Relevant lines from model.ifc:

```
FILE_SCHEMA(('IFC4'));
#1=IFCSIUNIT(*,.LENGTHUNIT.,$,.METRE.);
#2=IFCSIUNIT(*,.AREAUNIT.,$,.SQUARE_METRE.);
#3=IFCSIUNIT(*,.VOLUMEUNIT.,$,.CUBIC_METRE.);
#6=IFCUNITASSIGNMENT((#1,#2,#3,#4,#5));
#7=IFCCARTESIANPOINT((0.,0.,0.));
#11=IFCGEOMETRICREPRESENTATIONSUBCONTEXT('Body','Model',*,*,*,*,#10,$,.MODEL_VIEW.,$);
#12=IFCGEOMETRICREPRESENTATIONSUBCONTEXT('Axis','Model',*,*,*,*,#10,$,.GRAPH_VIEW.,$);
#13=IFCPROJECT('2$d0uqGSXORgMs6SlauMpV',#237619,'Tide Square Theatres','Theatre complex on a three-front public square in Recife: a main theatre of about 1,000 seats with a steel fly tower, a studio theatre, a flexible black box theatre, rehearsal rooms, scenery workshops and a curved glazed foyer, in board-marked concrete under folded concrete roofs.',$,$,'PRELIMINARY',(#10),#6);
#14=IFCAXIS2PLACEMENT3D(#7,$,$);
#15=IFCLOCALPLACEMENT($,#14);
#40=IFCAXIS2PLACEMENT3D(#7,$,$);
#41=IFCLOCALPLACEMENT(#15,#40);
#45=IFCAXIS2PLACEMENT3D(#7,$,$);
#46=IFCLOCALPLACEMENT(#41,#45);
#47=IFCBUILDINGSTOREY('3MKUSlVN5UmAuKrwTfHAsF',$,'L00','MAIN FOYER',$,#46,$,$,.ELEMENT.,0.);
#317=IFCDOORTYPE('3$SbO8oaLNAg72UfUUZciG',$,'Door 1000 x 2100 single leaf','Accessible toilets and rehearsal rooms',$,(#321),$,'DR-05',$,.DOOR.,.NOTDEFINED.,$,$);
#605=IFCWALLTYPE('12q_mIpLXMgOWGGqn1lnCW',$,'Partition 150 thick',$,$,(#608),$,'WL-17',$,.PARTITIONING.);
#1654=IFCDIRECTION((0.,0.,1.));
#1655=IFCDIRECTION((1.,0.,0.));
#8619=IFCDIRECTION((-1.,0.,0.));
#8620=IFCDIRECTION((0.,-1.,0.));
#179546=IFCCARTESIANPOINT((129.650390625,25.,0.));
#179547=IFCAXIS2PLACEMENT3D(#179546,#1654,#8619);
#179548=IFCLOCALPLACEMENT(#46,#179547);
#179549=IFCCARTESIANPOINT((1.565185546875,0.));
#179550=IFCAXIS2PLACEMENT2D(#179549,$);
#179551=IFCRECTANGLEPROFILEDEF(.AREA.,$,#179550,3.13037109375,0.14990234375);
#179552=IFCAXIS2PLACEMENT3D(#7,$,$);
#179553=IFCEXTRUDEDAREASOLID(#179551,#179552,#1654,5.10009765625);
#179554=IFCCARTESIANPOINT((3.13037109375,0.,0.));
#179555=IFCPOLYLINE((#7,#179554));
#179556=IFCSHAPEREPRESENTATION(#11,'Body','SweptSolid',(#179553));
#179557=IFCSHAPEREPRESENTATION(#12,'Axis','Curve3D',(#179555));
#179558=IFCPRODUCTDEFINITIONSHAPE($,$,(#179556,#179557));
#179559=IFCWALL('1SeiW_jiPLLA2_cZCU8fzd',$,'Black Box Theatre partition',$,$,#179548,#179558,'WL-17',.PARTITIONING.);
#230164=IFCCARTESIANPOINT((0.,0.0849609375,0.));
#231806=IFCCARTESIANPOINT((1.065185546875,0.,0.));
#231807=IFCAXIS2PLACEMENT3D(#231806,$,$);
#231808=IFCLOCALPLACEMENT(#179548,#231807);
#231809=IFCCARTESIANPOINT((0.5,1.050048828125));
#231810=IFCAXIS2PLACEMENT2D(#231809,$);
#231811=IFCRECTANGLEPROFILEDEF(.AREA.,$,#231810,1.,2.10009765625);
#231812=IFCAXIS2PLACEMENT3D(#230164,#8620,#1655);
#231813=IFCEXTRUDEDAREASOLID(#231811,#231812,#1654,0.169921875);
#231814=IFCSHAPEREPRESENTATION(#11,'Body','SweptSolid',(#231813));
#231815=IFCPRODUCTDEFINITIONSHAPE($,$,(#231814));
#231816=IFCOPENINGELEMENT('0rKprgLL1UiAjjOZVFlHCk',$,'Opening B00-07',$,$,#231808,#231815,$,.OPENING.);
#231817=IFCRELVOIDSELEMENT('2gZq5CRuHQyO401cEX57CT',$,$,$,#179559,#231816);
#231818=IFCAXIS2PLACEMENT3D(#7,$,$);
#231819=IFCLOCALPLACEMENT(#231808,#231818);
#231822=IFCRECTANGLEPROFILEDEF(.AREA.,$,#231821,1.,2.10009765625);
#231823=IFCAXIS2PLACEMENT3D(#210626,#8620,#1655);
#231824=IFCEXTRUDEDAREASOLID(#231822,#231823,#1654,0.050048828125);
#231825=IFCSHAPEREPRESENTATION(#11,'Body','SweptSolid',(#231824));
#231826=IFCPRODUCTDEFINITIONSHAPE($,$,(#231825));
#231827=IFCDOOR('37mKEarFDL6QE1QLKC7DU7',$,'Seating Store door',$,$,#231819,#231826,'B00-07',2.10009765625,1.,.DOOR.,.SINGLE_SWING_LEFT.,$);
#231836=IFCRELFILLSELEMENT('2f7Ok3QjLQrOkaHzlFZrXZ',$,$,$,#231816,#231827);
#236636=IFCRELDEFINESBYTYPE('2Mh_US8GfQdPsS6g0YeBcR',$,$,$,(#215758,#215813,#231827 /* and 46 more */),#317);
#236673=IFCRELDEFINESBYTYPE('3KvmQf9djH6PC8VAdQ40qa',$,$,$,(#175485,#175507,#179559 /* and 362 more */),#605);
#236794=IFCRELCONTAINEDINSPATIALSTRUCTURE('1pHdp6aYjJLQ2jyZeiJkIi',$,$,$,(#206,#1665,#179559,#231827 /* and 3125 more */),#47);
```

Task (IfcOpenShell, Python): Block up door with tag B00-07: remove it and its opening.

```python
import ifcopenshell
import ifcopenshell.api.feature
import ifcopenshell.api.root
import ifcopenshell.geom
import ifcopenshell.util.shape

model = ifcopenshell.open("model.ifc")
settings = ifcopenshell.geom.settings()


def volume(element):
    """Net volume in cubic metres, openings subtracted."""
    shape = ifcopenshell.geom.create_shape(settings, element)
    return ifcopenshell.util.shape.get_volume(shape.geometry)


door = model.by_guid("37mKEarFDL6QE1QLKC7DU7")
opening = door.FillsVoids[0].RelatingOpeningElement
wall = opening.VoidsElements[0].RelatingBuildingElement
before = volume(wall)

ifcopenshell.api.root.remove_product(model, product=door)
ifcopenshell.api.feature.remove_feature(model, feature=opening)

after = volume(wall)

print(f"wall volume {before:.3f} -> {after:.3f} m3")

model.write("model_edited.ifc")
```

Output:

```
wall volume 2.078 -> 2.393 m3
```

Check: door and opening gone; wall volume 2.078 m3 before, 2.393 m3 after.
